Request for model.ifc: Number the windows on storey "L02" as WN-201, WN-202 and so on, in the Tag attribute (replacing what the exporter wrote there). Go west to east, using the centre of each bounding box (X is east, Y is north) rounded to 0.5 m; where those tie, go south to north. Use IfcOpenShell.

First a look at what the model holds.

```python
import ifcopenshell
import ifcopenshell.util.element
import ifcopenshell.util.placement

model = ifcopenshell.open("model.ifc")
print(model.schema)
storey = next(s for s in model.by_type("IfcBuildingStorey") if s.Name == "L02")
windows = [e for e in ifcopenshell.util.element.get_decomposition(storey) if e.is_a("IfcWindow")]
for e in sorted(windows, key=lambda e: e.id()):
    origin = ifcopenshell.util.placement.get_local_placement(e.ObjectPlacement)[:3, 3]
    print(e.id(), e.Tag, e.Name, origin.round(2) + 0.0, sep=" | ")
```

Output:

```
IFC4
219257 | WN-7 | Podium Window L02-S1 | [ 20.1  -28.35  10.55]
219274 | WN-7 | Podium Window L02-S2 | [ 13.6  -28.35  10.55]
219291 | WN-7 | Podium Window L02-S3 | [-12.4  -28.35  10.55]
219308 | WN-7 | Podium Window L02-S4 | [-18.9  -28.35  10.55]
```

```python
import ifcopenshell
import ifcopenshell.geom
import ifcopenshell.util.element
import ifcopenshell.util.shape

model = ifcopenshell.open("model.ifc")
settings = ifcopenshell.geom.settings()
settings.set("use-world-coords", True)


def centre(element):
    shape = ifcopenshell.geom.create_shape(settings, element)
    return ifcopenshell.util.shape.get_bbox_centroid(shape.geometry)


storey = next(s for s in model.by_type("IfcBuildingStorey") if s.Name == "L02")
windows = [e for e in ifcopenshell.util.element.get_decomposition(storey) if e.is_a("IfcWindow")]

# Insertion points can sit at a corner or the storey origin, so sort by the geometry (in metres).
centres = {e: centre(e) for e in windows}
windows.sort(key=lambda e: (round(centres[e][0] / 0.5), centres[e][1]))

for i, e in enumerate(windows, start=1):
    number = f"WN-2{i:02d}"
    e.Tag = number
    print(e.id(), number)

model.write("model_v2.ifc")
```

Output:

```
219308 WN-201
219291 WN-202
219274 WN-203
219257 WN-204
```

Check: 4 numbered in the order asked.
